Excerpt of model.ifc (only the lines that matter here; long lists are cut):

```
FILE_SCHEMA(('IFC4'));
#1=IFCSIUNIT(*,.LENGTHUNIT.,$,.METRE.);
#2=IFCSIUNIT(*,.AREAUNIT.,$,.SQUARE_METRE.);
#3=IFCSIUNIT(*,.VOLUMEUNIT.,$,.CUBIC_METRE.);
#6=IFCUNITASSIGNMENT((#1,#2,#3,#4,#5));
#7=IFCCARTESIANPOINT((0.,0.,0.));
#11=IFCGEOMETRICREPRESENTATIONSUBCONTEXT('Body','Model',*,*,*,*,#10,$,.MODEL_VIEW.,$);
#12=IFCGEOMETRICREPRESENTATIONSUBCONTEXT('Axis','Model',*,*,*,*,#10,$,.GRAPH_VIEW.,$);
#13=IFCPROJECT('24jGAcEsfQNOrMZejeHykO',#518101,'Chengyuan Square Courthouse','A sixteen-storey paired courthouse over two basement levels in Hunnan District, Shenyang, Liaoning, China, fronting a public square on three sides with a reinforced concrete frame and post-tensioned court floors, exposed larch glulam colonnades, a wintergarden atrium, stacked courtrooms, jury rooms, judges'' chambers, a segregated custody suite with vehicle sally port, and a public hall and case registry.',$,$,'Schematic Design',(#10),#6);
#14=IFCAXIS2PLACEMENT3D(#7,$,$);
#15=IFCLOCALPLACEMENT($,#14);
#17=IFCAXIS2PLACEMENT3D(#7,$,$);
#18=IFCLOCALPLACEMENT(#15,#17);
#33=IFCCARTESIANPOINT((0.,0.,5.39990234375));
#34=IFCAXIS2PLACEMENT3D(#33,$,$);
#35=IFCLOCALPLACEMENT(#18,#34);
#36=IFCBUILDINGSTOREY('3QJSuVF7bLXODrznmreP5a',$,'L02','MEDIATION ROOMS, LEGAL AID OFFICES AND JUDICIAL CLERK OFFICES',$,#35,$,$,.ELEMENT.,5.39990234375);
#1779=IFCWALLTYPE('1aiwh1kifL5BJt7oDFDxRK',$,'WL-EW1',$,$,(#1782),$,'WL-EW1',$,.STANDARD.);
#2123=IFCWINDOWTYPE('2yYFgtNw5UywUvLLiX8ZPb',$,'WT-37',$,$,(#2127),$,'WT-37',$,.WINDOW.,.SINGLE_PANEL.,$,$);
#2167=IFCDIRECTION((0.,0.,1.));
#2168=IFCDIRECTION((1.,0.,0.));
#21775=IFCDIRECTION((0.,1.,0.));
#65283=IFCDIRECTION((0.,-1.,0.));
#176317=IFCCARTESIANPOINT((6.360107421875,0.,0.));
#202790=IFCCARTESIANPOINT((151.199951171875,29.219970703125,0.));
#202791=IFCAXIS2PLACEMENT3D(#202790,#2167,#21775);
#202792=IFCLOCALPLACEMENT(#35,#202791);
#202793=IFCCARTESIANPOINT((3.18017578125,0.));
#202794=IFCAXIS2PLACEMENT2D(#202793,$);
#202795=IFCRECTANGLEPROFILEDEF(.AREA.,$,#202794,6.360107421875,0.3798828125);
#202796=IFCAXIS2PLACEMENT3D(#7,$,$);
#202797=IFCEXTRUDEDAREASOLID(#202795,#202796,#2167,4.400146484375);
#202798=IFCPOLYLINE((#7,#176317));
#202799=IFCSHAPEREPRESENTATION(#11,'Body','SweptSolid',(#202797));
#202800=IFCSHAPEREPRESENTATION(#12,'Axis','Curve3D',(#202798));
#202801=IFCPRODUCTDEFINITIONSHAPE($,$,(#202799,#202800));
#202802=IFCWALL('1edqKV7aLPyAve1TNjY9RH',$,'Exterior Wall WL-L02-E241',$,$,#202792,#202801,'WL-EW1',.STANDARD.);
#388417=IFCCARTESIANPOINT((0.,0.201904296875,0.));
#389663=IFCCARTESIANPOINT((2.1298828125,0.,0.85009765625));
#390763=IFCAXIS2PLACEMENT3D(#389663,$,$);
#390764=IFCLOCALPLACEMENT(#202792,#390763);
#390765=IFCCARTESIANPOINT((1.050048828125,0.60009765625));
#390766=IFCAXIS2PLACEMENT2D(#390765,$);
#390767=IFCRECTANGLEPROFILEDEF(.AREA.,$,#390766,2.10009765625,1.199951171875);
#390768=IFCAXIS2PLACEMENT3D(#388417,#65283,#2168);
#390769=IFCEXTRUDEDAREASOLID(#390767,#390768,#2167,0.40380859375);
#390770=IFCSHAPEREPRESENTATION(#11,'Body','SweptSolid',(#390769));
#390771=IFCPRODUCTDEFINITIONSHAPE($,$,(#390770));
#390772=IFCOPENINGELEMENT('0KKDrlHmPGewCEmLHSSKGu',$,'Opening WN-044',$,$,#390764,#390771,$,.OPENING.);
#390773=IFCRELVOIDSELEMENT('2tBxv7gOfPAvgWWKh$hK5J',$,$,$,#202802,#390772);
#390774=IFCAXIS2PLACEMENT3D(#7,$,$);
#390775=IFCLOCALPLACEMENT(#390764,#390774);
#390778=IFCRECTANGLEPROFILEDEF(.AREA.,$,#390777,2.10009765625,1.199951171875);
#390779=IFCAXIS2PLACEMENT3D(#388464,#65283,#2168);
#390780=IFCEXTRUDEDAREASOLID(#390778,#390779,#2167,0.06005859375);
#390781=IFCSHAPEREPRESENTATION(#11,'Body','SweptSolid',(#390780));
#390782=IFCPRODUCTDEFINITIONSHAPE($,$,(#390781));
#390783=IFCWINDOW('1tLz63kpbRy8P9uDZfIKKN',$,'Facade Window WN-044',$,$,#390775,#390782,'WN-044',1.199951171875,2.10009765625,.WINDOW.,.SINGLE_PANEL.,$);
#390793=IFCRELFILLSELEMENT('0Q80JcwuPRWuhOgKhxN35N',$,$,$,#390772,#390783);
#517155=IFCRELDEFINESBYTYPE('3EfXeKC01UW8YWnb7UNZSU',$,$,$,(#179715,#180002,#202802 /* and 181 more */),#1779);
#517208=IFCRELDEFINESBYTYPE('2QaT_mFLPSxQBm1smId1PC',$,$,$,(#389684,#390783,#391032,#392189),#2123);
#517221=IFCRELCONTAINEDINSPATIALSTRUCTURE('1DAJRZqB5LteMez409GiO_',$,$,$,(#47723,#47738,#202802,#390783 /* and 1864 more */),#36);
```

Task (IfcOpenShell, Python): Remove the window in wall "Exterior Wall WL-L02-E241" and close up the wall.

```python
import ifcopenshell
import ifcopenshell.api.feature
import ifcopenshell.api.root
import ifcopenshell.geom
import ifcopenshell.util.shape

model = ifcopenshell.open("model.ifc")
settings = ifcopenshell.geom.settings()


def volume(element):
    """Net volume in cubic metres, openings subtracted."""
    shape = ifcopenshell.geom.create_shape(settings, element)
    return ifcopenshell.util.shape.get_volume(shape.geometry)


window = model.by_guid("1tLz63kpbRy8P9uDZfIKKN")
opening = window.FillsVoids[0].RelatingOpeningElement
wall = opening.VoidsElements[0].RelatingBuildingElement
before = volume(wall)

ifcopenshell.api.root.remove_product(model, product=window)
ifcopenshell.api.feature.remove_feature(model, feature=opening)

after = volume(wall)

print(f"wall volume {before:.3f} -> {after:.3f} m3")

model.write("model_v2.ifc")
```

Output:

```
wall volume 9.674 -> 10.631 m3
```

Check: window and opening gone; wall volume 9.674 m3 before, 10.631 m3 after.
